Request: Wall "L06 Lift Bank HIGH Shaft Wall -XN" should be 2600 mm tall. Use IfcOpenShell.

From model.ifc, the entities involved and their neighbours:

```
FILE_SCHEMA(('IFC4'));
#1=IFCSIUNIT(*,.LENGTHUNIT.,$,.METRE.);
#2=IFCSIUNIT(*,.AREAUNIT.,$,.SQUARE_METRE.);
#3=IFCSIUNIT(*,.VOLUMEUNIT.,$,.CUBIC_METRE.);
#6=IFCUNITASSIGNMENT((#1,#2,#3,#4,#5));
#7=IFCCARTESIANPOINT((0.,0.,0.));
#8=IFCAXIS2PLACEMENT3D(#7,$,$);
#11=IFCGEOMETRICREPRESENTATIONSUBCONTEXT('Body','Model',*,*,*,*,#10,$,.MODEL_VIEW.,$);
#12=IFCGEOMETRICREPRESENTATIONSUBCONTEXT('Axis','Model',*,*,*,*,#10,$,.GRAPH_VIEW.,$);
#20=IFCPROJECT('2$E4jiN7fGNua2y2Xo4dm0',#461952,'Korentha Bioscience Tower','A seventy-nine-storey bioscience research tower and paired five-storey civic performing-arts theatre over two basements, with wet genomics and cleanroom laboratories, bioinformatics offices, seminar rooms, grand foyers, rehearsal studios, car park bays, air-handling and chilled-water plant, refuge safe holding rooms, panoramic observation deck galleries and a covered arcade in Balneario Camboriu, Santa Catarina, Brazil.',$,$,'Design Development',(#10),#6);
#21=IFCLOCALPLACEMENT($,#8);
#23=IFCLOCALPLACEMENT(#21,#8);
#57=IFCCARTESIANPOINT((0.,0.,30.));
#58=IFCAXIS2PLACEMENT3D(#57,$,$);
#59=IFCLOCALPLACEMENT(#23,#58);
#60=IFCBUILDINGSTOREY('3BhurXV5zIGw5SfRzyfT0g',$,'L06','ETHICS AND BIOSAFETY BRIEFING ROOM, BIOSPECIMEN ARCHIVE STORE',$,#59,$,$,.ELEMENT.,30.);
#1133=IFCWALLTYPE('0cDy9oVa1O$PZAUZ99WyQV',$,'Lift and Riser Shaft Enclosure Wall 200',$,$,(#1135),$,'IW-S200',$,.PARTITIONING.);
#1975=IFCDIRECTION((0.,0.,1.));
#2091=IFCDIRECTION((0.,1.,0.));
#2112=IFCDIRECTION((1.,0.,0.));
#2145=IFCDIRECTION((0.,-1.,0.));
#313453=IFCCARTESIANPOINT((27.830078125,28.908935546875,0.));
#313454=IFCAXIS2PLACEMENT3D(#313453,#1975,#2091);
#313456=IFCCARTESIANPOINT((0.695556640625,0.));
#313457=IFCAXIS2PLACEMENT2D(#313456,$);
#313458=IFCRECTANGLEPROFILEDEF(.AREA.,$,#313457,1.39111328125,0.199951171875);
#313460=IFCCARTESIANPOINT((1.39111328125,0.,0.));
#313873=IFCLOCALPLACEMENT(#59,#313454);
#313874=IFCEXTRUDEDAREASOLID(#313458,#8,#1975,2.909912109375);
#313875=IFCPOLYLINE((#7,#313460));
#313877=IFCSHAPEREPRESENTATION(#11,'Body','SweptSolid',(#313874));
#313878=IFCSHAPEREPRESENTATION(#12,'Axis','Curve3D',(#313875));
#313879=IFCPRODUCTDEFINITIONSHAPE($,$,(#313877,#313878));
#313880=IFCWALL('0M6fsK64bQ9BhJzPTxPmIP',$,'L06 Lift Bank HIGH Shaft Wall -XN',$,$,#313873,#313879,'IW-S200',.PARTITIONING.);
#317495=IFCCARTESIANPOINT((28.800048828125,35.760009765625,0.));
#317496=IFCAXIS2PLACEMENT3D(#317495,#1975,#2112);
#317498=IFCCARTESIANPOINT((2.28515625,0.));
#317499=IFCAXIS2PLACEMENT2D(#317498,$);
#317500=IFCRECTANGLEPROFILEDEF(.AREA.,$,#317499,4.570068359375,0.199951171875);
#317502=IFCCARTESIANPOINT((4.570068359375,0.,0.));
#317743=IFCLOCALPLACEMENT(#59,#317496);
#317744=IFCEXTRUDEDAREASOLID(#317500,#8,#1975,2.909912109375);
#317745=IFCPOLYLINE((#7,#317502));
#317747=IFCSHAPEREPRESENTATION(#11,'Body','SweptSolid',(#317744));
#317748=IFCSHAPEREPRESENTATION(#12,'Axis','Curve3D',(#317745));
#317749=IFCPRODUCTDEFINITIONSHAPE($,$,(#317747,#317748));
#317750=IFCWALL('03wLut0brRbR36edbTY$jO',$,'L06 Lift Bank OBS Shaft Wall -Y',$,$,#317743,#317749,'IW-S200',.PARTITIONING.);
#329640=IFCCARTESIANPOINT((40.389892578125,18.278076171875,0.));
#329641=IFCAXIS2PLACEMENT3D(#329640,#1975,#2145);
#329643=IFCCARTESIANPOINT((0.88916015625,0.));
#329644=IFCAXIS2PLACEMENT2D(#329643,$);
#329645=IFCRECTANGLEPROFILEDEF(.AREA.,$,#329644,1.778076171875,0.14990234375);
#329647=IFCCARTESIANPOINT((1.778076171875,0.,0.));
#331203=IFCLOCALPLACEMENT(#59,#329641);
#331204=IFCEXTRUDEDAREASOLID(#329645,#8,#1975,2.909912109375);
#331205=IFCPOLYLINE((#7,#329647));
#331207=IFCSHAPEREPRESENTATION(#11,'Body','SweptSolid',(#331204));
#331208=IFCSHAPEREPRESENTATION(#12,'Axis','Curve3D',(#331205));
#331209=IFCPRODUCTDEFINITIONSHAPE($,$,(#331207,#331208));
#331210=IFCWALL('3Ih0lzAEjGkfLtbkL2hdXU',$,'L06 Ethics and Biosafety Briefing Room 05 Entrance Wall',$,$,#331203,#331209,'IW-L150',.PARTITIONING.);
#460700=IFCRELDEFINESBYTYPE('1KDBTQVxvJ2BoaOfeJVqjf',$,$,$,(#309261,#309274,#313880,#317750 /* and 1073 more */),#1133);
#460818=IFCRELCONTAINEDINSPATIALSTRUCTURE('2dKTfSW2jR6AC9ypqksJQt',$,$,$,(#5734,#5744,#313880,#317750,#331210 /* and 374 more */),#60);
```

```python
import ifcopenshell
import ifcopenshell.geom
import ifcopenshell.util.representation
import ifcopenshell.util.shape
import ifcopenshell.util.unit

model = ifcopenshell.open("model.ifc")
unit_scale = ifcopenshell.util.unit.calculate_unit_scale(model)
settings = ifcopenshell.geom.settings()


def volume(element):
    """Net volume in cubic metres, openings subtracted."""
    shape = ifcopenshell.geom.create_shape(settings, element)
    return ifcopenshell.util.shape.get_volume(shape.geometry)


wall = model.by_id(313880)
before = volume(wall)

body = ifcopenshell.util.representation.get_representation(wall, "Model", "Body")
solid = body.Items[0]
old_height = solid.Depth
solid.Depth = 2.6 / unit_scale
after = volume(wall)

print(f"height {old_height:g} -> {solid.Depth:g}, volume {before:.3f} -> {after:.3f} m3")

model.write("model_updated.ifc")
```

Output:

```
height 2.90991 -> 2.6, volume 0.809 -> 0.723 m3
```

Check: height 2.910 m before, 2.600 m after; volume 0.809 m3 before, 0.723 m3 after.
